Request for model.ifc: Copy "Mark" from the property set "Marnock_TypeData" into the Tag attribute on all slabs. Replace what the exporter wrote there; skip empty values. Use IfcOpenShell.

First a look at what the model holds.

```python
import ifcopenshell
import ifcopenshell.util.element

model = ifcopenshell.open("model.ifc")
print(model.schema)
slabs = model.by_type("IfcSlab")
print(len(slabs), "slabs")
for e in slabs[:8]:
    source = ifcopenshell.util.element.get_pset(e, "Marnock_TypeData", "Mark")
    target = e.Tag
    print(e.id(), repr(source), repr(target), sep=" | ")
```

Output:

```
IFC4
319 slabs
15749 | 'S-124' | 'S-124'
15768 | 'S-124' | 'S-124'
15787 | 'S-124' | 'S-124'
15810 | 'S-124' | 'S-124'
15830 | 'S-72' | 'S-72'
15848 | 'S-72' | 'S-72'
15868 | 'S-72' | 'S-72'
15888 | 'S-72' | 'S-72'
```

```python
import ifcopenshell
import ifcopenshell.util.element

model = ifcopenshell.open("model.ifc")

count = 0
for e in model.by_type("IfcSlab"):
    value = ifcopenshell.util.element.get_pset(e, "Marnock_TypeData", "Mark")
    current = e.Tag
    if not value or not value.strip() or current == value:
        continue
    e.Tag = value
    count += 1

print(count, "slabs updated")

model.write("model_edited.ifc")
```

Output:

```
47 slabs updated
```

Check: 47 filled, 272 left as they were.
